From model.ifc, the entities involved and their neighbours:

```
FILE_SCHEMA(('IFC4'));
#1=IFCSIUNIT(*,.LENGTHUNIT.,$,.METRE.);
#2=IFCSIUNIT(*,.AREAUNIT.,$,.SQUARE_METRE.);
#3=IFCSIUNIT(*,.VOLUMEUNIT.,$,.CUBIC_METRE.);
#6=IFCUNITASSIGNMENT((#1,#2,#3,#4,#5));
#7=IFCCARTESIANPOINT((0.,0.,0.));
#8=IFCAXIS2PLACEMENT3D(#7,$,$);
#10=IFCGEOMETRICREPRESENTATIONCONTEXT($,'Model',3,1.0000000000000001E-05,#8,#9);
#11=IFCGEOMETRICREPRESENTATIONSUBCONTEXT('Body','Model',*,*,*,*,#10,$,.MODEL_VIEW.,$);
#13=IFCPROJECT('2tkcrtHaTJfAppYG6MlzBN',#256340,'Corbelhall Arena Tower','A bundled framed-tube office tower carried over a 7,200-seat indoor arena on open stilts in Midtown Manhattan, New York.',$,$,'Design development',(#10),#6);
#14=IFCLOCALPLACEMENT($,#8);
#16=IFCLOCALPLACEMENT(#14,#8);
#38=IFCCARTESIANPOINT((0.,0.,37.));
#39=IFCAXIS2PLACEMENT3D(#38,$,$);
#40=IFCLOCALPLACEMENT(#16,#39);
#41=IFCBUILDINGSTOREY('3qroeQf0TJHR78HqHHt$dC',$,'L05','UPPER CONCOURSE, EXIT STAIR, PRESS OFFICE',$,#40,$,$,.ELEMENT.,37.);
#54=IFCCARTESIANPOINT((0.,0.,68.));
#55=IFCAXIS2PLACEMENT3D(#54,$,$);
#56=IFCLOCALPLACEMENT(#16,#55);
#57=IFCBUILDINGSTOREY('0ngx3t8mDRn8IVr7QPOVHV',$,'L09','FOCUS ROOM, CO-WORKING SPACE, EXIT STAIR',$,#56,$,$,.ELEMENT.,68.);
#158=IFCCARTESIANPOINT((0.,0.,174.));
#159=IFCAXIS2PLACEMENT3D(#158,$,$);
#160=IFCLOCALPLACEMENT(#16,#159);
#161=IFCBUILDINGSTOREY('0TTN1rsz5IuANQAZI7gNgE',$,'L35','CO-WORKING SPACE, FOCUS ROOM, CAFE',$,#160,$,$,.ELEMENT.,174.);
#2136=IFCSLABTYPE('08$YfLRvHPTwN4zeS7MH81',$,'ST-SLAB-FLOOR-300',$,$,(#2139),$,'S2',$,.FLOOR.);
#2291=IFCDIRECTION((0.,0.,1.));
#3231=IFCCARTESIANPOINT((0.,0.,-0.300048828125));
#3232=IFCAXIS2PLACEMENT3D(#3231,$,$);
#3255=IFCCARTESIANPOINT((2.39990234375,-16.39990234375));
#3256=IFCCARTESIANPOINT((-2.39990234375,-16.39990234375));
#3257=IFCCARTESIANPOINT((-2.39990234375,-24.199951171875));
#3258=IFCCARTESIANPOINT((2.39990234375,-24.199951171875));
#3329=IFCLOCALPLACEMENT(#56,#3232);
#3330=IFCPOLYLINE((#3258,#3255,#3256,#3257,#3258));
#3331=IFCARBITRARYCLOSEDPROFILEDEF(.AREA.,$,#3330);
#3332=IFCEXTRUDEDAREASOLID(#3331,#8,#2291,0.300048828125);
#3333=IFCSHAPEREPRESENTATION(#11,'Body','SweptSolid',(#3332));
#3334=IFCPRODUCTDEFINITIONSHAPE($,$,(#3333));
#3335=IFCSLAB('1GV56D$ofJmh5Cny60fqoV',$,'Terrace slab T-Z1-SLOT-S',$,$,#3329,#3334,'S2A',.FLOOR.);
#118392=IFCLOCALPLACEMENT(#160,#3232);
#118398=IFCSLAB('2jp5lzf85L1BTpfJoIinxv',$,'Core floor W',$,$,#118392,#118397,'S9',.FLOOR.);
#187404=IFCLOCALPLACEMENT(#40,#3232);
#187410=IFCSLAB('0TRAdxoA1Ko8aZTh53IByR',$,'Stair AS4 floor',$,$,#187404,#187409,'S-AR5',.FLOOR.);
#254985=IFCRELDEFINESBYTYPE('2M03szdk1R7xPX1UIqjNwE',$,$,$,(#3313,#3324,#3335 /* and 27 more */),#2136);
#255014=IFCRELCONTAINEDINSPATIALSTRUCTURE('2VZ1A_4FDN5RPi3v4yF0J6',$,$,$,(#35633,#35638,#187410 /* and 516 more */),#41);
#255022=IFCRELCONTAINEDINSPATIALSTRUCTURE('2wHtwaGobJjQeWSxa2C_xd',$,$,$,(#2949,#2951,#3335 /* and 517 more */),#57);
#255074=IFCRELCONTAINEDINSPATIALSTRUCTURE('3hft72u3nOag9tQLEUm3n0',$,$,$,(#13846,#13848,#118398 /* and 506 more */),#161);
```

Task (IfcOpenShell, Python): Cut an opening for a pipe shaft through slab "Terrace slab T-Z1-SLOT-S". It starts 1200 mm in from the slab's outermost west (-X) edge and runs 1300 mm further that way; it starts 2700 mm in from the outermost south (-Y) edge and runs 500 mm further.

```python
import numpy as np
import ifcopenshell
import ifcopenshell.api.feature
import ifcopenshell.api.geometry
import ifcopenshell.api.root
import ifcopenshell.geom
import ifcopenshell.util.placement
import ifcopenshell.util.representation
import ifcopenshell.util.shape
import ifcopenshell.util.unit

model = ifcopenshell.open("model.ifc")
unit_scale = ifcopenshell.util.unit.calculate_unit_scale(model)
settings = ifcopenshell.geom.settings()


def volume(element):
    """Net volume in cubic metres, openings subtracted."""
    shape = ifcopenshell.geom.create_shape(settings, element)
    return ifcopenshell.util.shape.get_volume(shape.geometry)


slab = model.by_guid("1GV56D$ofJmh5Cny60fqoV")
before = volume(slab)

# Extent in the slab's own axes, in metres. The edges named are its -X and -Y sides.
slab_shape = ifcopenshell.geom.create_shape(settings, slab)
vertices = ifcopenshell.util.shape.get_vertices(slab_shape.geometry)
x_min, y_min, bottom = vertices.min(axis=0)
top = vertices[:, 2].max()

opening = ifcopenshell.api.root.create_entity(model, ifc_class="IfcOpeningElement", name="Pipe shaft opening", predefined_type="OPENING")
context = ifcopenshell.util.representation.get_context(model, "Model", "Body", "MODEL_VIEW")
width, depth = 1.3, 0.5
outline = [(0.0, 0.0), (width, 0.0), (width, depth), (0.0, depth), (0.0, 0.0)]
# Overshoot both faces by 50 mm so the cut is clean.
shape = ifcopenshell.api.geometry.add_slab_representation(
    model, context=context, depth=top - bottom + 0.1, polyline=outline
)
ifcopenshell.api.geometry.assign_representation(model, product=opening, representation=shape)

matrix = ifcopenshell.util.placement.get_local_placement(slab.ObjectPlacement)
matrix[:, 3] = matrix @ np.append(np.array([x_min + 1.2, y_min + 2.7, bottom - 0.05]) / unit_scale, 1.0)
ifcopenshell.api.geometry.edit_object_placement(model, product=opening, matrix=matrix, is_si=False)
ifcopenshell.api.feature.add_feature(model, feature=opening, element=slab)

after = volume(slab)

print(f"slab volume {before:.3f} -> {after:.3f} m3")

model.write("model_v2.ifc")
```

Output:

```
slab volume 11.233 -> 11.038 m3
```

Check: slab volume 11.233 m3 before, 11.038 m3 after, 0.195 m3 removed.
